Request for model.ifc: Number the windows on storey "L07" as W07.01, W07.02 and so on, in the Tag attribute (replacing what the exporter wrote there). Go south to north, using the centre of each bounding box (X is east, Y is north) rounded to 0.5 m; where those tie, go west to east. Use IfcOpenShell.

First a look at what the model holds.

```python
import ifcopenshell
import ifcopenshell.util.element
import ifcopenshell.util.placement

model = ifcopenshell.open("model.ifc")
print(model.schema)
storey = next(s for s in model.by_type("IfcBuildingStorey") if s.Name == "L07")
windows = [e for e in ifcopenshell.util.element.get_decomposition(storey) if e.is_a("IfcWindow")]
for e in sorted(windows, key=lambda e: e.id()):
    origin = ifcopenshell.util.placement.get_local_placement(e.ObjectPlacement)[:3, 3]
    print(e.id(), e.Tag, e.Name, origin.round(2) + 0.0, sep=" | ")
```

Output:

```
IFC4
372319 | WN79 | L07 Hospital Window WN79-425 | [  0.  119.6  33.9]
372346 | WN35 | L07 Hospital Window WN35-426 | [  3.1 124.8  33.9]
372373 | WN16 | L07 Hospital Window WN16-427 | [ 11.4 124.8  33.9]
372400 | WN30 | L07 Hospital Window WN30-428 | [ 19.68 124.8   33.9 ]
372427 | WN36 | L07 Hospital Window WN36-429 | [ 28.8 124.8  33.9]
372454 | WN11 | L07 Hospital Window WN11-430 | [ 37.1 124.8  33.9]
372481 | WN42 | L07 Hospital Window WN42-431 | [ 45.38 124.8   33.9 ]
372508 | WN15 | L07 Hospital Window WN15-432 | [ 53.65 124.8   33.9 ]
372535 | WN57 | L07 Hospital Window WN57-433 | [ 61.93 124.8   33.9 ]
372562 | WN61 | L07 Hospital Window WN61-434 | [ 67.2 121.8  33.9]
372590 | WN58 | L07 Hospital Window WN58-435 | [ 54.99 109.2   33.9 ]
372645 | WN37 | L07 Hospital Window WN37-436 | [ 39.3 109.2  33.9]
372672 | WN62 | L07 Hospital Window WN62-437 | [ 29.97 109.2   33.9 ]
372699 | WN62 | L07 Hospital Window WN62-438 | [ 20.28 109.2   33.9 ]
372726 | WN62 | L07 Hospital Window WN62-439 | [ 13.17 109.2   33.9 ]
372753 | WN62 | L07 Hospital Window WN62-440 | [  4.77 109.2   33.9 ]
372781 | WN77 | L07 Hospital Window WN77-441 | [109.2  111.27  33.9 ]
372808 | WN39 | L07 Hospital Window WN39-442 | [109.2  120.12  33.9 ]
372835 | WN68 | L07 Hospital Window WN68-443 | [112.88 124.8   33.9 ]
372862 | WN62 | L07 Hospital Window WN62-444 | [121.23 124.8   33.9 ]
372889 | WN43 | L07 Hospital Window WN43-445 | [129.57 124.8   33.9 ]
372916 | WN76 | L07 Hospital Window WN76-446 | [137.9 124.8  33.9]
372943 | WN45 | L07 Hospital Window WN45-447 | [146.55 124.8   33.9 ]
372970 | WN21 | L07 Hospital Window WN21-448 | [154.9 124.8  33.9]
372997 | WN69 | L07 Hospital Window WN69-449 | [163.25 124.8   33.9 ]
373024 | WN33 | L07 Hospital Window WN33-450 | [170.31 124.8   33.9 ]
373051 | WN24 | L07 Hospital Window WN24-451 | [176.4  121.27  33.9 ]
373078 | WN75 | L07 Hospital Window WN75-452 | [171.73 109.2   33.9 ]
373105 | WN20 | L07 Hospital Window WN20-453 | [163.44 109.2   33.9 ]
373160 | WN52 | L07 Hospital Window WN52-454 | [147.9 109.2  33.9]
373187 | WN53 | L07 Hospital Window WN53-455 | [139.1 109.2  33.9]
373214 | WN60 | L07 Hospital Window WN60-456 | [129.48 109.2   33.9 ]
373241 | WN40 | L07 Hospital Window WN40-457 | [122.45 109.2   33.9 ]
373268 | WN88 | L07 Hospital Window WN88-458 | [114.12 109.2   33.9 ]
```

```python
import ifcopenshell
import ifcopenshell.geom
import ifcopenshell.util.element
import ifcopenshell.util.shape

model = ifcopenshell.open("model.ifc")
settings = ifcopenshell.geom.settings()
settings.set("use-world-coords", True)


def centre(element):
    shape = ifcopenshell.geom.create_shape(settings, element)
    return ifcopenshell.util.shape.get_bbox_centroid(shape.geometry)


storey = next(s for s in model.by_type("IfcBuildingStorey") if s.Name == "L07")
windows = [e for e in ifcopenshell.util.element.get_decomposition(storey) if e.is_a("IfcWindow")]

# Insertion points can sit at a corner or the storey origin, so sort by the geometry (in metres).
centres = {e: centre(e) for e in windows}
windows.sort(key=lambda e: (round(centres[e][1] / 0.5), centres[e][0]))

for i, e in enumerate(windows, start=1):
    number = f"W07.{i:02d}"
    e.Tag = number
    print(e.id(), number)

model.write("model-out.ifc")
```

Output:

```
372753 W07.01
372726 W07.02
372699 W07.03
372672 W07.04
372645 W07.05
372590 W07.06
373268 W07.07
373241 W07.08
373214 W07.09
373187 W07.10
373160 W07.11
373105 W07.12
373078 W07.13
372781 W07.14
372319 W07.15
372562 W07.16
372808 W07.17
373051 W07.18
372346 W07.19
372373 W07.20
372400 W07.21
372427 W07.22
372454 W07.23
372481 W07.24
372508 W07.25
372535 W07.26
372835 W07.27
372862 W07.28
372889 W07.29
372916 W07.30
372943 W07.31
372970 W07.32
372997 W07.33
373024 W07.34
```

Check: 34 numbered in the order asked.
